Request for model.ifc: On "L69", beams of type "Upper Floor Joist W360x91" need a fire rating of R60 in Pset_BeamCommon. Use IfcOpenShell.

First a look at what the model holds.

```python
import ifcopenshell
import ifcopenshell.util.element

model = ifcopenshell.open("model.ifc")
print(model.schema)
storey = next(s for s in model.by_type("IfcBuildingStorey") if s.Name == "L69")
beams = [e for e in ifcopenshell.util.element.get_decomposition(storey) if e.is_a("IfcBeam")]
seen = {}
for e in beams:
    element_type = ifcopenshell.util.element.get_type(e)
    key = (element_type.Name if element_type != e and element_type else None, ifcopenshell.util.element.get_pset(e, "Pset_BeamCommon", "FireRating"))
    seen[key] = seen.get(key, 0) + 1
for (name, value), count in sorted(seen.items(), key=str):
    print(count, "x", name, "|", value)
```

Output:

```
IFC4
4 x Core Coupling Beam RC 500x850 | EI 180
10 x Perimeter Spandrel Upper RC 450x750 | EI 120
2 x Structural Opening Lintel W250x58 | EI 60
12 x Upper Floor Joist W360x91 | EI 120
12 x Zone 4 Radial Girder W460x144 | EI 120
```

```python
import ifcopenshell
import ifcopenshell.api.pset
import ifcopenshell.util.element

model = ifcopenshell.open("model.ifc")

storey = next(s for s in model.by_type("IfcBuildingStorey") if s.Name == "L69")
beams = [e for e in ifcopenshell.util.element.get_decomposition(storey) if e.is_a("IfcBeam")]

count = 0
for e in beams:
    element_type = ifcopenshell.util.element.get_type(e)
    if element_type in (None, e) or element_type.Name != "Upper Floor Joist W360x91":
        continue
    found = ifcopenshell.util.element.get_pset(e, "Pset_BeamCommon", should_inherit=False)
    if found:
        pset = model.by_id(found["id"])
        if len(ifcopenshell.util.element.get_elements_by_pset(pset)) > 1:
            pset = ifcopenshell.api.pset.unshare_pset(model, products=[e], pset=pset)[0]
    else:
        pset = ifcopenshell.api.pset.add_pset(model, product=e, name="Pset_BeamCommon")
    ifcopenshell.api.pset.edit_pset(model, pset=pset, properties={"FireRating": "R60"})
    count += 1

print(count, "beams updated")

model.write("model_rev.ifc")
```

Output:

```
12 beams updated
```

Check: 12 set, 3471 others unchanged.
